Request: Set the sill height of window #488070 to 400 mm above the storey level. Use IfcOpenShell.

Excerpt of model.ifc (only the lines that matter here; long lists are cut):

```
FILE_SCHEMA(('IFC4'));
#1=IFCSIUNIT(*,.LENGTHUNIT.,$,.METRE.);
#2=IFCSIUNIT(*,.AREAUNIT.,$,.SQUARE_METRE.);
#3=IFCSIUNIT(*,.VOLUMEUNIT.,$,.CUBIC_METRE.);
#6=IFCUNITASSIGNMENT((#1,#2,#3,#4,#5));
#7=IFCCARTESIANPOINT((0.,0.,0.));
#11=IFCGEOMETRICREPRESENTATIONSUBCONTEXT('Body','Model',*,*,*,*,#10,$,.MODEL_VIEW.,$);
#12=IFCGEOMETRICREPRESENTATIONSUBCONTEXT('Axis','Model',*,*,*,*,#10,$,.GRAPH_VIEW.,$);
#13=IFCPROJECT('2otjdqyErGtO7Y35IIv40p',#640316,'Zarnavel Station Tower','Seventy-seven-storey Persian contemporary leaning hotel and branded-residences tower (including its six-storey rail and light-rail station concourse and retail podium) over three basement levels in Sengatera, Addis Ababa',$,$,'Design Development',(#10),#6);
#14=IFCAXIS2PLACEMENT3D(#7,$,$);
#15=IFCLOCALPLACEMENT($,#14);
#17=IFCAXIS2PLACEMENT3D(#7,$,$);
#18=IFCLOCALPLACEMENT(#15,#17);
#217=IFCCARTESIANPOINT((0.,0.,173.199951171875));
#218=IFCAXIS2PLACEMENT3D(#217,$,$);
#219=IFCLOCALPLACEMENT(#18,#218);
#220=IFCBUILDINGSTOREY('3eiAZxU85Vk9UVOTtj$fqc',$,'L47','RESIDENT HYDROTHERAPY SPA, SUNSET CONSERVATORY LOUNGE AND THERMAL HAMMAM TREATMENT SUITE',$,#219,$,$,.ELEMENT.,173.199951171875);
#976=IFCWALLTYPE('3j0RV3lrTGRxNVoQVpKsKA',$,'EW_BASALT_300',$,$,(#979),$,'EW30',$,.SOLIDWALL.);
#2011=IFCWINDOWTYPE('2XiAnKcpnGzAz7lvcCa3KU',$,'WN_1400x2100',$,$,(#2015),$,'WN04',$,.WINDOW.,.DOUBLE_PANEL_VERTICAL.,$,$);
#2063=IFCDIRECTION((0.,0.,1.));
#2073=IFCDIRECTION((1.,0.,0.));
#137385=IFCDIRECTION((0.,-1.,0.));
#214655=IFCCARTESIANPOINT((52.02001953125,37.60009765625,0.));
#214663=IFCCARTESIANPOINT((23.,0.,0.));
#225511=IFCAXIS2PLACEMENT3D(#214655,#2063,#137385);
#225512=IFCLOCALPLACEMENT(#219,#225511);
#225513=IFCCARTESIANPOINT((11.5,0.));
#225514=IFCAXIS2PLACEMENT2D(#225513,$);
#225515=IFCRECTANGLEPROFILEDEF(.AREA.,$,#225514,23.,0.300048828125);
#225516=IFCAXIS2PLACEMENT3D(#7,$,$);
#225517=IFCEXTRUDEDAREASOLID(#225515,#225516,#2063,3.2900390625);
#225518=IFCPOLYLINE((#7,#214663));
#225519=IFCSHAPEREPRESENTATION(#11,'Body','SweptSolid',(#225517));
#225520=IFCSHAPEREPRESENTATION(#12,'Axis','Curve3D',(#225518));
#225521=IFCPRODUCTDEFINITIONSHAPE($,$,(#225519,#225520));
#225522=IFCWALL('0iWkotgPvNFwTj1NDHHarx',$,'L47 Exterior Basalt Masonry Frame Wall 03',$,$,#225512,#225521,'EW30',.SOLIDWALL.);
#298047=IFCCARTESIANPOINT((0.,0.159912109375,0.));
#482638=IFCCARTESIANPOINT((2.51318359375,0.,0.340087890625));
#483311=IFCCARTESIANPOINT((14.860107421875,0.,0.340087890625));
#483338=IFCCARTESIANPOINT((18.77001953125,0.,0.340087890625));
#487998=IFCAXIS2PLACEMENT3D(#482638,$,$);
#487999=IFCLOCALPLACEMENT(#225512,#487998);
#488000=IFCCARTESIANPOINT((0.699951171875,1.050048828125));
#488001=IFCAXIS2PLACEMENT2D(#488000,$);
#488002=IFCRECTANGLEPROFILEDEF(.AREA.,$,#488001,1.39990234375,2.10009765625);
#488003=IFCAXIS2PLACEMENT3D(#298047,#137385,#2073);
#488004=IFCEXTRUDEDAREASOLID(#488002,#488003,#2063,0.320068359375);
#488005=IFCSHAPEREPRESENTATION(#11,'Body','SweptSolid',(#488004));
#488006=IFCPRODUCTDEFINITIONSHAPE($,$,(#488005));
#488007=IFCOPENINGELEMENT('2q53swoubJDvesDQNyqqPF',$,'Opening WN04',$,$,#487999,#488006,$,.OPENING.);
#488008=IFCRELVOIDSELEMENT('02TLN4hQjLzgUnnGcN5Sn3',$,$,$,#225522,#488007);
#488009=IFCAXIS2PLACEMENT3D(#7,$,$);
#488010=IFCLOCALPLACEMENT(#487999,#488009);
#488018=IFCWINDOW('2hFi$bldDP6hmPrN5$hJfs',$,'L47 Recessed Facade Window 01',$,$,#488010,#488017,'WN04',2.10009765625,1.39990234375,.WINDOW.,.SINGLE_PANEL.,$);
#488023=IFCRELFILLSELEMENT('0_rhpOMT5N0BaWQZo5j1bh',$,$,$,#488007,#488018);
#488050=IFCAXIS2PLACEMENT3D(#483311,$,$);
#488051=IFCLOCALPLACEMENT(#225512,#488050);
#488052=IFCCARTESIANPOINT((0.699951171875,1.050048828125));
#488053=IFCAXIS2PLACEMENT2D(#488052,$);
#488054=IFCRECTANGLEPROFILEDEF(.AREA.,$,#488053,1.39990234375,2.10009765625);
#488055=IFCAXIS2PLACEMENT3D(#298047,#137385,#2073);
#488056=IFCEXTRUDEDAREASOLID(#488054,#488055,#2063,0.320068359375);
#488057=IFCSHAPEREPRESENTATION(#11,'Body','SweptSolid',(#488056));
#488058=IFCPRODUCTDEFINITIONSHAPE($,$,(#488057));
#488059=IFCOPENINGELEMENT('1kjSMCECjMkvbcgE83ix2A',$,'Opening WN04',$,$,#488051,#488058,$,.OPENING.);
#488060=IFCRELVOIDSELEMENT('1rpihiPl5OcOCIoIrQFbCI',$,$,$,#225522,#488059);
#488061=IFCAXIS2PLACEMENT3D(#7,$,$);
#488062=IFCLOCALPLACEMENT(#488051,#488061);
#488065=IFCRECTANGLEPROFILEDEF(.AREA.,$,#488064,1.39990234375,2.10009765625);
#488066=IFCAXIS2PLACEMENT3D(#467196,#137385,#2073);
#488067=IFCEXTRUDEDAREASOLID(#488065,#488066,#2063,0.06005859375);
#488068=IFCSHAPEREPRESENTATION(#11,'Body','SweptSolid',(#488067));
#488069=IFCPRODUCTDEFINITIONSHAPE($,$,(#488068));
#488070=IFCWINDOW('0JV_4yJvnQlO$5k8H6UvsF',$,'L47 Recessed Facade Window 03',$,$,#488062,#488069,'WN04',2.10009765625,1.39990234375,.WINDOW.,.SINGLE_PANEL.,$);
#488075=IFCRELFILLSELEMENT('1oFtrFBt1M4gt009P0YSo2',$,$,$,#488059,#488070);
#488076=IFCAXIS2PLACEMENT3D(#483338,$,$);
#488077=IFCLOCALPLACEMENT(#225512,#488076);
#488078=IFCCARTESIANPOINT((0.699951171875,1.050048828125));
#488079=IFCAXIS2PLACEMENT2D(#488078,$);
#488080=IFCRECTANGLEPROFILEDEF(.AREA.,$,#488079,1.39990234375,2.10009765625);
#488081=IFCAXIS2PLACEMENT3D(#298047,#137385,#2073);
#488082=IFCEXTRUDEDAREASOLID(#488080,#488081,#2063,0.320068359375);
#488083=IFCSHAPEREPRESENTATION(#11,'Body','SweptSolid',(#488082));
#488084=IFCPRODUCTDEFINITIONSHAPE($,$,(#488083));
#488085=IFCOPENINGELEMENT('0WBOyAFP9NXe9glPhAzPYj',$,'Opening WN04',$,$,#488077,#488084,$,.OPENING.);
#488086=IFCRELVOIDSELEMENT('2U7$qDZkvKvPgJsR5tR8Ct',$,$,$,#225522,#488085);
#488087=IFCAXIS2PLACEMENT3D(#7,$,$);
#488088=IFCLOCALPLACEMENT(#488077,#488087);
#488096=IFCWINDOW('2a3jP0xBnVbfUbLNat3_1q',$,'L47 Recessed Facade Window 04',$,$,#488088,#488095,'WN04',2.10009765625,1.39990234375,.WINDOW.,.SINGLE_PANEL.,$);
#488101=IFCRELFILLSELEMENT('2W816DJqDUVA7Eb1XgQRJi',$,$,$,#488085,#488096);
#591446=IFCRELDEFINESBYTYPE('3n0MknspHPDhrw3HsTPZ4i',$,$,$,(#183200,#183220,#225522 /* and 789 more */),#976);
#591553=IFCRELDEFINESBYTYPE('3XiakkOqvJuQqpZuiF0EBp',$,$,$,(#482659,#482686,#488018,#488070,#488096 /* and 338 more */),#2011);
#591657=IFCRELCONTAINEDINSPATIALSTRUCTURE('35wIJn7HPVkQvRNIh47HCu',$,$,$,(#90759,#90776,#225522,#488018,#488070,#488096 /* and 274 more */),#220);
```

```python
import numpy as np
import ifcopenshell
import ifcopenshell.api.geometry
import ifcopenshell.geom
import ifcopenshell.util.element
import ifcopenshell.util.placement
import ifcopenshell.util.shape
import ifcopenshell.util.unit

model = ifcopenshell.open("model.ifc")
unit_scale = ifcopenshell.util.unit.calculate_unit_scale(model)

window = model.by_guid("0JV_4yJvnQlO$5k8H6UvsF")
opening = window.FillsVoids[0].RelatingOpeningElement
storey = ifcopenshell.util.element.get_container(window, ifc_class="IfcBuildingStorey")
level = ifcopenshell.util.placement.get_local_placement(storey.ObjectPlacement)[2, 3]

# The opening's origin need not be at the sill, so measure its lowest point.
shape = ifcopenshell.geom.create_shape(ifcopenshell.geom.settings(), opening)
bottom = ifcopenshell.util.shape.get_shape_bottom_elevation(shape, shape.geometry) / unit_scale
dz = level + 0.4 - bottom

shift = np.array([0.0, 0.0, dz])
# The window is placed relative to its opening, so it follows when the opening moves.
matrix = ifcopenshell.util.placement.get_local_placement(opening.ObjectPlacement)
matrix[:3, 3] += shift
ifcopenshell.api.geometry.edit_object_placement(
    model, product=opening, matrix=matrix, is_si=False, should_transform_children=True
)

print(f"moved by {dz * unit_scale:+.3f} m")

model.write("model_v2.ifc")
```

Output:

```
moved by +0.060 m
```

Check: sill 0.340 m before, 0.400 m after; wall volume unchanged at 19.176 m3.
